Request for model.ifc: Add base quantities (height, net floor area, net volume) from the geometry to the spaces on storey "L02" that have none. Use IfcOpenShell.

First a look at what the model holds.

```python
import ifcopenshell
import ifcopenshell.util.element
import ifcopenshell.util.unit

model = ifcopenshell.open("model.ifc")
print(model.schema)
for unit_type in ("LENGTHUNIT", "AREAUNIT", "VOLUMEUNIT"):
    print(unit_type, ifcopenshell.util.unit.calculate_unit_scale(model, unit_type))
storey = next(s for s in model.by_type("IfcBuildingStorey") if s.Name == "L02")
spaces = [e for e in ifcopenshell.util.element.get_decomposition(storey) if e.is_a("IfcSpace")]
for e in sorted(spaces, key=lambda e: e.id()):
    print(e.id(), e.is_a(), e.Name, list(ifcopenshell.util.element.get_psets(e, qtos_only=True)), sep=" | ")
```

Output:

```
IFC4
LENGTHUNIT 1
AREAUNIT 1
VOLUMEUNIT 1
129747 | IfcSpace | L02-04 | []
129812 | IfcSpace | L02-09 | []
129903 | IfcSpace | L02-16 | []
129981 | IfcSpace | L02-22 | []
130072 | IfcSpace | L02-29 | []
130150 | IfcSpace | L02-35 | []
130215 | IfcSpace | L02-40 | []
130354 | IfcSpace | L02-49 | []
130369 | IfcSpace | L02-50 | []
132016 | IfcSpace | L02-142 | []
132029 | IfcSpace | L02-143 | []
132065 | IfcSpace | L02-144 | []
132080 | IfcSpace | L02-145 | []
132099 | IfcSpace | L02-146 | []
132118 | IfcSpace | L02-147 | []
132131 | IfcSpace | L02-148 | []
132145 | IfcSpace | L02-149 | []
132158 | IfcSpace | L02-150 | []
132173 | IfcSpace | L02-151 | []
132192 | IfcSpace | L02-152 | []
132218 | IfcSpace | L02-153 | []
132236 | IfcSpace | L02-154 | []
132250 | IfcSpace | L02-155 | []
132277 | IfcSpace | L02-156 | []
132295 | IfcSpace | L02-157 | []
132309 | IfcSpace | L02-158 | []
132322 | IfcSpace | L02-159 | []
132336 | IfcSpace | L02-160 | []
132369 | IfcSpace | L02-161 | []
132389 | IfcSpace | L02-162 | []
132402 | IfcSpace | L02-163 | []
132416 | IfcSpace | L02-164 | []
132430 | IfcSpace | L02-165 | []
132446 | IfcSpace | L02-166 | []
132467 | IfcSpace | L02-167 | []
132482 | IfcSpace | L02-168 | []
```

```python
import ifcopenshell
import ifcopenshell.api.pset
import ifcopenshell.geom
import ifcopenshell.util.element
import ifcopenshell.util.shape
import ifcopenshell.util.unit

model = ifcopenshell.open("model.ifc")
unit_scale = ifcopenshell.util.unit.calculate_unit_scale(model)
area_scale = ifcopenshell.util.unit.calculate_unit_scale(model, "AREAUNIT")
volume_scale = ifcopenshell.util.unit.calculate_unit_scale(model, "VOLUMEUNIT")
settings = ifcopenshell.geom.settings()

storey = next(s for s in model.by_type("IfcBuildingStorey") if s.Name == "L02")
spaces = [e for e in ifcopenshell.util.element.get_decomposition(storey) if e.is_a("IfcSpace")]

for e in sorted(spaces, key=lambda e: e.id()):
    if ifcopenshell.util.element.get_psets(e, qtos_only=True, should_inherit=False):
        continue
    # Geometry comes back in metres, in the element's own axes.
    shape = ifcopenshell.geom.create_shape(settings, e)
    values = {
        "Height": ifcopenshell.util.shape.get_z(shape.geometry) / unit_scale,
        "NetFloorArea": ifcopenshell.util.shape.get_footprint_area(shape.geometry) / area_scale,
        "NetVolume": ifcopenshell.util.shape.get_volume(shape.geometry) / volume_scale,
    }
    qto = ifcopenshell.api.pset.add_qto(model, product=e, name="Qto_SpaceBaseQuantities")
    ifcopenshell.api.pset.edit_qto(model, qto=qto, properties=values)
    print(e.id(), {k: round(v, 3) for k, v in values.items()})

model.write("model_v2.ifc")
```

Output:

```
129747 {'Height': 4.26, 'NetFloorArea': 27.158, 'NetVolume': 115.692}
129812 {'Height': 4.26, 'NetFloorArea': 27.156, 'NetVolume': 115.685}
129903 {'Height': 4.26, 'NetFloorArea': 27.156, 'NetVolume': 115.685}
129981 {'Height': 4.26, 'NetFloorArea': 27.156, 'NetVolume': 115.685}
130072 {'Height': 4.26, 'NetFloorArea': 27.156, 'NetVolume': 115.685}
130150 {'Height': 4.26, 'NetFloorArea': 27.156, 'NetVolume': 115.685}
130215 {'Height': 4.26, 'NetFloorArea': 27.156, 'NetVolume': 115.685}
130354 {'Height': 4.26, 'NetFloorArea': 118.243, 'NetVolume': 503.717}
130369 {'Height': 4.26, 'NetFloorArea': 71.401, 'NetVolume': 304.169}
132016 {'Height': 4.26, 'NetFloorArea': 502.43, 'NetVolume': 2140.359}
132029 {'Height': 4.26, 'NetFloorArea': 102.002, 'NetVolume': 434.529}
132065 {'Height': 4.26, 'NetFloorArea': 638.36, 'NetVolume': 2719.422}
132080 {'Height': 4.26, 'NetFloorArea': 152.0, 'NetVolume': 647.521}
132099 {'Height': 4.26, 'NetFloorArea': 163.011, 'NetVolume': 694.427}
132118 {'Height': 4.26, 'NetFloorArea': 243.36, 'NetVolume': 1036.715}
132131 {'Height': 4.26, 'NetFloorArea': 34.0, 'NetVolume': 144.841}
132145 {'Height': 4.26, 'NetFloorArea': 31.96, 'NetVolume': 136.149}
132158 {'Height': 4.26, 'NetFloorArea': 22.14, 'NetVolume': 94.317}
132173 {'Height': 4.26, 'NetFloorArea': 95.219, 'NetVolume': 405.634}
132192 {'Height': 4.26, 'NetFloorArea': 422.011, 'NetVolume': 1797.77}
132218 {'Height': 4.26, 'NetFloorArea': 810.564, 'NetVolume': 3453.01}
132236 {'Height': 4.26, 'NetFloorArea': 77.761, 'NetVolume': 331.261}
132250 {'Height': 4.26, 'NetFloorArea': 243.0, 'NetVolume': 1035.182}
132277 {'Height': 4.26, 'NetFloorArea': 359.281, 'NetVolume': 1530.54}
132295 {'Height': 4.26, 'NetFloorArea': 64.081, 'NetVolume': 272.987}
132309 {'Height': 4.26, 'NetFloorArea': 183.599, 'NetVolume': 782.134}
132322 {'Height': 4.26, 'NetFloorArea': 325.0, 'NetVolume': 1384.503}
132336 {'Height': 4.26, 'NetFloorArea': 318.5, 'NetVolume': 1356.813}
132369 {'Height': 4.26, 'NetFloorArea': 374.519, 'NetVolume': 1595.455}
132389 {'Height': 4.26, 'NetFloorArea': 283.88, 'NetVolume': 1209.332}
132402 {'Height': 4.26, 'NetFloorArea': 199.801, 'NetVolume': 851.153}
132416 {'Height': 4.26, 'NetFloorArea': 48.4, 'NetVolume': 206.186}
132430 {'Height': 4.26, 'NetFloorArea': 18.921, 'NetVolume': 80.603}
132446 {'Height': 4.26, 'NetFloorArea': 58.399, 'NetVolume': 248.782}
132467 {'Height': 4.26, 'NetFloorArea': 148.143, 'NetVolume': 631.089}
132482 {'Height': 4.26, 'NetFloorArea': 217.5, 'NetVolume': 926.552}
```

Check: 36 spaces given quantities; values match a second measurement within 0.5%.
